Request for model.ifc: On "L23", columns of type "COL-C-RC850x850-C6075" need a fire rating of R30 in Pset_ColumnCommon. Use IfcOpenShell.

First a look at what the model holds.

```python
import ifcopenshell
import ifcopenshell.util.element

model = ifcopenshell.open("model.ifc")
print(model.schema)
storey = next(s for s in model.by_type("IfcBuildingStorey") if s.Name == "L23")
columns = [e for e in ifcopenshell.util.element.get_decomposition(storey) if e.is_a("IfcColumn")]
seen = {}
for e in columns:
    element_type = ifcopenshell.util.element.get_type(e)
    key = (element_type.Name if element_type != e and element_type else None, ifcopenshell.util.element.get_pset(e, "Pset_ColumnCommon", "FireRating"))
    seen[key] = seen.get(key, 0) + 1
for (name, value), count in sorted(seen.items(), key=str):
    print(count, "x", name, "|", value)
```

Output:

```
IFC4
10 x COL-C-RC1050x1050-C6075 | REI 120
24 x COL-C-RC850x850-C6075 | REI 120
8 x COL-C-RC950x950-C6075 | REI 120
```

```python
import ifcopenshell
import ifcopenshell.api.pset
import ifcopenshell.util.element

model = ifcopenshell.open("model.ifc")

storey = next(s for s in model.by_type("IfcBuildingStorey") if s.Name == "L23")
columns = [e for e in ifcopenshell.util.element.get_decomposition(storey) if e.is_a("IfcColumn")]

count = 0
for e in columns:
    element_type = ifcopenshell.util.element.get_type(e)
    if element_type in (None, e) or element_type.Name != "COL-C-RC850x850-C6075":
        continue
    found = ifcopenshell.util.element.get_pset(e, "Pset_ColumnCommon", should_inherit=False)
    if found:
        pset = model.by_id(found["id"])
        if len(ifcopenshell.util.element.get_elements_by_pset(pset)) > 1:
            pset = ifcopenshell.api.pset.unshare_pset(model, products=[e], pset=pset)[0]
    else:
        pset = ifcopenshell.api.pset.add_pset(model, product=e, name="Pset_ColumnCommon")
    ifcopenshell.api.pset.edit_pset(model, pset=pset, properties={"FireRating": "R30"})
    count += 1

print(count, "columns updated")

model.write("model-out.ifc")
```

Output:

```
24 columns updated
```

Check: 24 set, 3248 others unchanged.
